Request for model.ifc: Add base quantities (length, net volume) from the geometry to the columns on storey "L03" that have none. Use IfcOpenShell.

First a look at what the model holds.

```python
import ifcopenshell
import ifcopenshell.util.element
import ifcopenshell.util.unit

model = ifcopenshell.open("model.ifc")
print(model.schema)
for unit_type in ("LENGTHUNIT", "AREAUNIT", "VOLUMEUNIT"):
    print(unit_type, ifcopenshell.util.unit.calculate_unit_scale(model, unit_type))
storey = next(s for s in model.by_type("IfcBuildingStorey") if s.Name == "L03")
columns = [e for e in ifcopenshell.util.element.get_decomposition(storey) if e.is_a("IfcColumn")]
for e in sorted(columns, key=lambda e: e.id()):
    print(e.id(), e.is_a(), e.Name, list(ifcopenshell.util.element.get_psets(e, qtos_only=True)), sep=" | ")
```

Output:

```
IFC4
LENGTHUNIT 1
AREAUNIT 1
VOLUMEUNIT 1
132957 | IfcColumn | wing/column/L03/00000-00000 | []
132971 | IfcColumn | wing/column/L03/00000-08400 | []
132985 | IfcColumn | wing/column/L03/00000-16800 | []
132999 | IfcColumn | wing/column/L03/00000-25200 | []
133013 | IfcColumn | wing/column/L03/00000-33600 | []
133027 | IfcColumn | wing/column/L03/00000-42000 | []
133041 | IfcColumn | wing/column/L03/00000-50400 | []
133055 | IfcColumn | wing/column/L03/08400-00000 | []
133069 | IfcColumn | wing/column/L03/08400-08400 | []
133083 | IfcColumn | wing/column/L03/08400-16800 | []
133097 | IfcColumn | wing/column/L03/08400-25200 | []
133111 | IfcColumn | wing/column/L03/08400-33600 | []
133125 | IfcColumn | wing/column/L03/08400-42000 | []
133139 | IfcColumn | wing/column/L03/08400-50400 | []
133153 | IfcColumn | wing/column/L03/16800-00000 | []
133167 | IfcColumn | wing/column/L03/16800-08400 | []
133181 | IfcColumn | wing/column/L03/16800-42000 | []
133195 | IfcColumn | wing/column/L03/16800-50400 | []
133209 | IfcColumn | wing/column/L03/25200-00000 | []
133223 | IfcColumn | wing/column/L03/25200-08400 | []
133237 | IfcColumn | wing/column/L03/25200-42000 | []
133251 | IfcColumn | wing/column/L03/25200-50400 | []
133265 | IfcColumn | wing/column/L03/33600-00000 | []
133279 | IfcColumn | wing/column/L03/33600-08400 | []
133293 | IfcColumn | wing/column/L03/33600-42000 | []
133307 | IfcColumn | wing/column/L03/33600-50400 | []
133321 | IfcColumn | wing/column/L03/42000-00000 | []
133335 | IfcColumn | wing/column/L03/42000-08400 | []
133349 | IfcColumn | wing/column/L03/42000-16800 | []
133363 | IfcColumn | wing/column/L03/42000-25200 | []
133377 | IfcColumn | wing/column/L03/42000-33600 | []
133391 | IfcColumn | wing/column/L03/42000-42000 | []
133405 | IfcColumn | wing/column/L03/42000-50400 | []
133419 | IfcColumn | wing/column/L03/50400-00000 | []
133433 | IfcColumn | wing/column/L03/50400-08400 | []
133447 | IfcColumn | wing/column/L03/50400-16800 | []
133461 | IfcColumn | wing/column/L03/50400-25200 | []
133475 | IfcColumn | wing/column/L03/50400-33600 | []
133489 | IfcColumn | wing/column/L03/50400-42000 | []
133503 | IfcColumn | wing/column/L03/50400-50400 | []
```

```python
import ifcopenshell
import ifcopenshell.api.pset
import ifcopenshell.geom
import ifcopenshell.util.element
import ifcopenshell.util.shape
import ifcopenshell.util.unit

model = ifcopenshell.open("model.ifc")
unit_scale = ifcopenshell.util.unit.calculate_unit_scale(model)
volume_scale = ifcopenshell.util.unit.calculate_unit_scale(model, "VOLUMEUNIT")
settings = ifcopenshell.geom.settings()

storey = next(s for s in model.by_type("IfcBuildingStorey") if s.Name == "L03")
columns = [e for e in ifcopenshell.util.element.get_decomposition(storey) if e.is_a("IfcColumn")]

for e in sorted(columns, key=lambda e: e.id()):
    if ifcopenshell.util.element.get_psets(e, qtos_only=True, should_inherit=False):
        continue
    # Geometry comes back in metres, in the element's own axes.
    shape = ifcopenshell.geom.create_shape(settings, e)
    values = {
        "Length": ifcopenshell.util.shape.get_z(shape.geometry) / unit_scale,
        "NetVolume": ifcopenshell.util.shape.get_volume(shape.geometry) / volume_scale,
    }
    qto = ifcopenshell.api.pset.add_qto(model, product=e, name="Qto_ColumnBaseQuantities")
    ifcopenshell.api.pset.edit_qto(model, qto=qto, properties=values)
    print(e.id(), {k: round(v, 3) for k, v in values.items()})

model.write("model_v2.ifc")
```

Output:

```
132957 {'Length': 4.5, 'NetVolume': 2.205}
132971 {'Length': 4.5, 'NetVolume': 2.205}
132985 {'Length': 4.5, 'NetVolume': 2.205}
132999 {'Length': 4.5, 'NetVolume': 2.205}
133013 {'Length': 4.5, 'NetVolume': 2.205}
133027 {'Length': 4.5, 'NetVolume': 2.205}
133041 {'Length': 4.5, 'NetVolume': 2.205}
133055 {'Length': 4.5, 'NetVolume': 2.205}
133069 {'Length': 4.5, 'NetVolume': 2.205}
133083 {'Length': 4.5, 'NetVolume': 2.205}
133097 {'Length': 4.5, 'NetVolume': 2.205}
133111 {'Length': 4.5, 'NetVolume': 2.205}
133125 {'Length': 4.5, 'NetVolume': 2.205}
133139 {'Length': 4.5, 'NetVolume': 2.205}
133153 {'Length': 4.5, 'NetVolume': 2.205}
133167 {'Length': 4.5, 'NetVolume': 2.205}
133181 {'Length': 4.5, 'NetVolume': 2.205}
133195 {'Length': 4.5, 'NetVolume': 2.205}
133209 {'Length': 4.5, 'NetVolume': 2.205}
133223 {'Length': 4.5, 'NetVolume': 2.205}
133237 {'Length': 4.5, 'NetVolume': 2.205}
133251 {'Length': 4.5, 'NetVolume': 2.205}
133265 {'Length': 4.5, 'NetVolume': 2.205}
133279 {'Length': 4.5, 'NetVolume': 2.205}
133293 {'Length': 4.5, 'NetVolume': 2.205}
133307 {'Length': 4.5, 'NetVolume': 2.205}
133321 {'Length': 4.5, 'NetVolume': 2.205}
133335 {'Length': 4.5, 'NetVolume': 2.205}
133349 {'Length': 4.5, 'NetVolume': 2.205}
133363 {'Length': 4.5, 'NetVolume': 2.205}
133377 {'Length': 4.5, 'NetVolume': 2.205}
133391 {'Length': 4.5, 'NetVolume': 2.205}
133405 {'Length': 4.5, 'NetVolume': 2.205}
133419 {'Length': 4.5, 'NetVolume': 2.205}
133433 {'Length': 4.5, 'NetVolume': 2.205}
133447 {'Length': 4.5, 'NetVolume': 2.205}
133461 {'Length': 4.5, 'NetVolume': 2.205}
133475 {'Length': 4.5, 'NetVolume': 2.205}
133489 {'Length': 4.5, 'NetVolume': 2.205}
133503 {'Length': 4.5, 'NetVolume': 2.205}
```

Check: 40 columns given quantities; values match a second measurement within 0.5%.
